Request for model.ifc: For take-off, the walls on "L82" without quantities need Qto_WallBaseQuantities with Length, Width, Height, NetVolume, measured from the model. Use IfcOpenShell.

First a look at what the model holds.

```python
import ifcopenshell
import ifcopenshell.util.element
import ifcopenshell.util.unit

model = ifcopenshell.open("model.ifc")
print(model.schema)
for unit_type in ("LENGTHUNIT", "AREAUNIT", "VOLUMEUNIT"):
    print(unit_type, ifcopenshell.util.unit.calculate_unit_scale(model, unit_type))
storey = next(s for s in model.by_type("IfcBuildingStorey") if s.Name == "L82")
walls = [e for e in ifcopenshell.util.element.get_decomposition(storey) if e.is_a("IfcWall")]
for e in sorted(walls, key=lambda e: e.id()):
    print(e.id(), e.is_a(), e.Name, list(ifcopenshell.util.element.get_psets(e, qtos_only=True)), sep=" | ")
```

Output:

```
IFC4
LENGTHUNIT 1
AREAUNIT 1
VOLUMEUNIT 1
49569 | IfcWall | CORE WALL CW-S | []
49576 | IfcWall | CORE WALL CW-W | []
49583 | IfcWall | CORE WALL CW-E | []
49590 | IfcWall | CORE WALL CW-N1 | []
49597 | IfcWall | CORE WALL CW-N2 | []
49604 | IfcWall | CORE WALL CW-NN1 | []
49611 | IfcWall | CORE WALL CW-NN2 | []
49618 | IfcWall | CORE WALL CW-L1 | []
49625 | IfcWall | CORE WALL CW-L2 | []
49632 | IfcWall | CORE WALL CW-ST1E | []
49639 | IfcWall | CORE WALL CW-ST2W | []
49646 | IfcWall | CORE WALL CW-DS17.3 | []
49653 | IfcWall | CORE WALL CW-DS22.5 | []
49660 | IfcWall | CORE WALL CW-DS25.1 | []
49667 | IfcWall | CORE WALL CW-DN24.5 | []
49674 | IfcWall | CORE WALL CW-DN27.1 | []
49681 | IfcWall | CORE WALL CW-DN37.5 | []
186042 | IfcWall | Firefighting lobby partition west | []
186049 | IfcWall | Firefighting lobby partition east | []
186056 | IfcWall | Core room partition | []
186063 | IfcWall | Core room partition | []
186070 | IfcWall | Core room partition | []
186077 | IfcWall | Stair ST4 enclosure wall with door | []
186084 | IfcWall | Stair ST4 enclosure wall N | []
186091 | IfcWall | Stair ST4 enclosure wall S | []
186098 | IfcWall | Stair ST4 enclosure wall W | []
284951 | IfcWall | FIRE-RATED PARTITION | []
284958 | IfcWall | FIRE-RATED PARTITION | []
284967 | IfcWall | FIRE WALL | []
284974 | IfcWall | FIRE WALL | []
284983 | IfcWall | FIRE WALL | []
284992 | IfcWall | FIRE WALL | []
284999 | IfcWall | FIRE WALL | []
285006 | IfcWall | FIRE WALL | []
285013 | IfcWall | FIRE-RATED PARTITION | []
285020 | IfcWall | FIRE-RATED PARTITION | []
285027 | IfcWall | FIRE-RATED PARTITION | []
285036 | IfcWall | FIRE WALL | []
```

```python
import ifcopenshell
import ifcopenshell.api.pset
import ifcopenshell.geom
import ifcopenshell.util.element
import ifcopenshell.util.shape
import ifcopenshell.util.unit

model = ifcopenshell.open("model.ifc")
unit_scale = ifcopenshell.util.unit.calculate_unit_scale(model)
volume_scale = ifcopenshell.util.unit.calculate_unit_scale(model, "VOLUMEUNIT")
settings = ifcopenshell.geom.settings()

storey = next(s for s in model.by_type("IfcBuildingStorey") if s.Name == "L82")
walls = [e for e in ifcopenshell.util.element.get_decomposition(storey) if e.is_a("IfcWall")]

for e in sorted(walls, key=lambda e: e.id()):
    if ifcopenshell.util.element.get_psets(e, qtos_only=True, should_inherit=False):
        continue
    # Geometry comes back in metres, in the element's own axes.
    shape = ifcopenshell.geom.create_shape(settings, e)
    values = {
        "Length": ifcopenshell.util.shape.get_x(shape.geometry) / unit_scale,
        "Width": ifcopenshell.util.shape.get_y(shape.geometry) / unit_scale,
        "Height": ifcopenshell.util.shape.get_z(shape.geometry) / unit_scale,
        "NetVolume": ifcopenshell.util.shape.get_volume(shape.geometry) / volume_scale,
    }
    qto = ifcopenshell.api.pset.add_qto(model, product=e, name="Qto_WallBaseQuantities")
    ifcopenshell.api.pset.edit_qto(model, qto=qto, properties=values)
    print(e.id(), {k: round(v, 3) for k, v in values.items()})

model.write("model_edited.ifc")
```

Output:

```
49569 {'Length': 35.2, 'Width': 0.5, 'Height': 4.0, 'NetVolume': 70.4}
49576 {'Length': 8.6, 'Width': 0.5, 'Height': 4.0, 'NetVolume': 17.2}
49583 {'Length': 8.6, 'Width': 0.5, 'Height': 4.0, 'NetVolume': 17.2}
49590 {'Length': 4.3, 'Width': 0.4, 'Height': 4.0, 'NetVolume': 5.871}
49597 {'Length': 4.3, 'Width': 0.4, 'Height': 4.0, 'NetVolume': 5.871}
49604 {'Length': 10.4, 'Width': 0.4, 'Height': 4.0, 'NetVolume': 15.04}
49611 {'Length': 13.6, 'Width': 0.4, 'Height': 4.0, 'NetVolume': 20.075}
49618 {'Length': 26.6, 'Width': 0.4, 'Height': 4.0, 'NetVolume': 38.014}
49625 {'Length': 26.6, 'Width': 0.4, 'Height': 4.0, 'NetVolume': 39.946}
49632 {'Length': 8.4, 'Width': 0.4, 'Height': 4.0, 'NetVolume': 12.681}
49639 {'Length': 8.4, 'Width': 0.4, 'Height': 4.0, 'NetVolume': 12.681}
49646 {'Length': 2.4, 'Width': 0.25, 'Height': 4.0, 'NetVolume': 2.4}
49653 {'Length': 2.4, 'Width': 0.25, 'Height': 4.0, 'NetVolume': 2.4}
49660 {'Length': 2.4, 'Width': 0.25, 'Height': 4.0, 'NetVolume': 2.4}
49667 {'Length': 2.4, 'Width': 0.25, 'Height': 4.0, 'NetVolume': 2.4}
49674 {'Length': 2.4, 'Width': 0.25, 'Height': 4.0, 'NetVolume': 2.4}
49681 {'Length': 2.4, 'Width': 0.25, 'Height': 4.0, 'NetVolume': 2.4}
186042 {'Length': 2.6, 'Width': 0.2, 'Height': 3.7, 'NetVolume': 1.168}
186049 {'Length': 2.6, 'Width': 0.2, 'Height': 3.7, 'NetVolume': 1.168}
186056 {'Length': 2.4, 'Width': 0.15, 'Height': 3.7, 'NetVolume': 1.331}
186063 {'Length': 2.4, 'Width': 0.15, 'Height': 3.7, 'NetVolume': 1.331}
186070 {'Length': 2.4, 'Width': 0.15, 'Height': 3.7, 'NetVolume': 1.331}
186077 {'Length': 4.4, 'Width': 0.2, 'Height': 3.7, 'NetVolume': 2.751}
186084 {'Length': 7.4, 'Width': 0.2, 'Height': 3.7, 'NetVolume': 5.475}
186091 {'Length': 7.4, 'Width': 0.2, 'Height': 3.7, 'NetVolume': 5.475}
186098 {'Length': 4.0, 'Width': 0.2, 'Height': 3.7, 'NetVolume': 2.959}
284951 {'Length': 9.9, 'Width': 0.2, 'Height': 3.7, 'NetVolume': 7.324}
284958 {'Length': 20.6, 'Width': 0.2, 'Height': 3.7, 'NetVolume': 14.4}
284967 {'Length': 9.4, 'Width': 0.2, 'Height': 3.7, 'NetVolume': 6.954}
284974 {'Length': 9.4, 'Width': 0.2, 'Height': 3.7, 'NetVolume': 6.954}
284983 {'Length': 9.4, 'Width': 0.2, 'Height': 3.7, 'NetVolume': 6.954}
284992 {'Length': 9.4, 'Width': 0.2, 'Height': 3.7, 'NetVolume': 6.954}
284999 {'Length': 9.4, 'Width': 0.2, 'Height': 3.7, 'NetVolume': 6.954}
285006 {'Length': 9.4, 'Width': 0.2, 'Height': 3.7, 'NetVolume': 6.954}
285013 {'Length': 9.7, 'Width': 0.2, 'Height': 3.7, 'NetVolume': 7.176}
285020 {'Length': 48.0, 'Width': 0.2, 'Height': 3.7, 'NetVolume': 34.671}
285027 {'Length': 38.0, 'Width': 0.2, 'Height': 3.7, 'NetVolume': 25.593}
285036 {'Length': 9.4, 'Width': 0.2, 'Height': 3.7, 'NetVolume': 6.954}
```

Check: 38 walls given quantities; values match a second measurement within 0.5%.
